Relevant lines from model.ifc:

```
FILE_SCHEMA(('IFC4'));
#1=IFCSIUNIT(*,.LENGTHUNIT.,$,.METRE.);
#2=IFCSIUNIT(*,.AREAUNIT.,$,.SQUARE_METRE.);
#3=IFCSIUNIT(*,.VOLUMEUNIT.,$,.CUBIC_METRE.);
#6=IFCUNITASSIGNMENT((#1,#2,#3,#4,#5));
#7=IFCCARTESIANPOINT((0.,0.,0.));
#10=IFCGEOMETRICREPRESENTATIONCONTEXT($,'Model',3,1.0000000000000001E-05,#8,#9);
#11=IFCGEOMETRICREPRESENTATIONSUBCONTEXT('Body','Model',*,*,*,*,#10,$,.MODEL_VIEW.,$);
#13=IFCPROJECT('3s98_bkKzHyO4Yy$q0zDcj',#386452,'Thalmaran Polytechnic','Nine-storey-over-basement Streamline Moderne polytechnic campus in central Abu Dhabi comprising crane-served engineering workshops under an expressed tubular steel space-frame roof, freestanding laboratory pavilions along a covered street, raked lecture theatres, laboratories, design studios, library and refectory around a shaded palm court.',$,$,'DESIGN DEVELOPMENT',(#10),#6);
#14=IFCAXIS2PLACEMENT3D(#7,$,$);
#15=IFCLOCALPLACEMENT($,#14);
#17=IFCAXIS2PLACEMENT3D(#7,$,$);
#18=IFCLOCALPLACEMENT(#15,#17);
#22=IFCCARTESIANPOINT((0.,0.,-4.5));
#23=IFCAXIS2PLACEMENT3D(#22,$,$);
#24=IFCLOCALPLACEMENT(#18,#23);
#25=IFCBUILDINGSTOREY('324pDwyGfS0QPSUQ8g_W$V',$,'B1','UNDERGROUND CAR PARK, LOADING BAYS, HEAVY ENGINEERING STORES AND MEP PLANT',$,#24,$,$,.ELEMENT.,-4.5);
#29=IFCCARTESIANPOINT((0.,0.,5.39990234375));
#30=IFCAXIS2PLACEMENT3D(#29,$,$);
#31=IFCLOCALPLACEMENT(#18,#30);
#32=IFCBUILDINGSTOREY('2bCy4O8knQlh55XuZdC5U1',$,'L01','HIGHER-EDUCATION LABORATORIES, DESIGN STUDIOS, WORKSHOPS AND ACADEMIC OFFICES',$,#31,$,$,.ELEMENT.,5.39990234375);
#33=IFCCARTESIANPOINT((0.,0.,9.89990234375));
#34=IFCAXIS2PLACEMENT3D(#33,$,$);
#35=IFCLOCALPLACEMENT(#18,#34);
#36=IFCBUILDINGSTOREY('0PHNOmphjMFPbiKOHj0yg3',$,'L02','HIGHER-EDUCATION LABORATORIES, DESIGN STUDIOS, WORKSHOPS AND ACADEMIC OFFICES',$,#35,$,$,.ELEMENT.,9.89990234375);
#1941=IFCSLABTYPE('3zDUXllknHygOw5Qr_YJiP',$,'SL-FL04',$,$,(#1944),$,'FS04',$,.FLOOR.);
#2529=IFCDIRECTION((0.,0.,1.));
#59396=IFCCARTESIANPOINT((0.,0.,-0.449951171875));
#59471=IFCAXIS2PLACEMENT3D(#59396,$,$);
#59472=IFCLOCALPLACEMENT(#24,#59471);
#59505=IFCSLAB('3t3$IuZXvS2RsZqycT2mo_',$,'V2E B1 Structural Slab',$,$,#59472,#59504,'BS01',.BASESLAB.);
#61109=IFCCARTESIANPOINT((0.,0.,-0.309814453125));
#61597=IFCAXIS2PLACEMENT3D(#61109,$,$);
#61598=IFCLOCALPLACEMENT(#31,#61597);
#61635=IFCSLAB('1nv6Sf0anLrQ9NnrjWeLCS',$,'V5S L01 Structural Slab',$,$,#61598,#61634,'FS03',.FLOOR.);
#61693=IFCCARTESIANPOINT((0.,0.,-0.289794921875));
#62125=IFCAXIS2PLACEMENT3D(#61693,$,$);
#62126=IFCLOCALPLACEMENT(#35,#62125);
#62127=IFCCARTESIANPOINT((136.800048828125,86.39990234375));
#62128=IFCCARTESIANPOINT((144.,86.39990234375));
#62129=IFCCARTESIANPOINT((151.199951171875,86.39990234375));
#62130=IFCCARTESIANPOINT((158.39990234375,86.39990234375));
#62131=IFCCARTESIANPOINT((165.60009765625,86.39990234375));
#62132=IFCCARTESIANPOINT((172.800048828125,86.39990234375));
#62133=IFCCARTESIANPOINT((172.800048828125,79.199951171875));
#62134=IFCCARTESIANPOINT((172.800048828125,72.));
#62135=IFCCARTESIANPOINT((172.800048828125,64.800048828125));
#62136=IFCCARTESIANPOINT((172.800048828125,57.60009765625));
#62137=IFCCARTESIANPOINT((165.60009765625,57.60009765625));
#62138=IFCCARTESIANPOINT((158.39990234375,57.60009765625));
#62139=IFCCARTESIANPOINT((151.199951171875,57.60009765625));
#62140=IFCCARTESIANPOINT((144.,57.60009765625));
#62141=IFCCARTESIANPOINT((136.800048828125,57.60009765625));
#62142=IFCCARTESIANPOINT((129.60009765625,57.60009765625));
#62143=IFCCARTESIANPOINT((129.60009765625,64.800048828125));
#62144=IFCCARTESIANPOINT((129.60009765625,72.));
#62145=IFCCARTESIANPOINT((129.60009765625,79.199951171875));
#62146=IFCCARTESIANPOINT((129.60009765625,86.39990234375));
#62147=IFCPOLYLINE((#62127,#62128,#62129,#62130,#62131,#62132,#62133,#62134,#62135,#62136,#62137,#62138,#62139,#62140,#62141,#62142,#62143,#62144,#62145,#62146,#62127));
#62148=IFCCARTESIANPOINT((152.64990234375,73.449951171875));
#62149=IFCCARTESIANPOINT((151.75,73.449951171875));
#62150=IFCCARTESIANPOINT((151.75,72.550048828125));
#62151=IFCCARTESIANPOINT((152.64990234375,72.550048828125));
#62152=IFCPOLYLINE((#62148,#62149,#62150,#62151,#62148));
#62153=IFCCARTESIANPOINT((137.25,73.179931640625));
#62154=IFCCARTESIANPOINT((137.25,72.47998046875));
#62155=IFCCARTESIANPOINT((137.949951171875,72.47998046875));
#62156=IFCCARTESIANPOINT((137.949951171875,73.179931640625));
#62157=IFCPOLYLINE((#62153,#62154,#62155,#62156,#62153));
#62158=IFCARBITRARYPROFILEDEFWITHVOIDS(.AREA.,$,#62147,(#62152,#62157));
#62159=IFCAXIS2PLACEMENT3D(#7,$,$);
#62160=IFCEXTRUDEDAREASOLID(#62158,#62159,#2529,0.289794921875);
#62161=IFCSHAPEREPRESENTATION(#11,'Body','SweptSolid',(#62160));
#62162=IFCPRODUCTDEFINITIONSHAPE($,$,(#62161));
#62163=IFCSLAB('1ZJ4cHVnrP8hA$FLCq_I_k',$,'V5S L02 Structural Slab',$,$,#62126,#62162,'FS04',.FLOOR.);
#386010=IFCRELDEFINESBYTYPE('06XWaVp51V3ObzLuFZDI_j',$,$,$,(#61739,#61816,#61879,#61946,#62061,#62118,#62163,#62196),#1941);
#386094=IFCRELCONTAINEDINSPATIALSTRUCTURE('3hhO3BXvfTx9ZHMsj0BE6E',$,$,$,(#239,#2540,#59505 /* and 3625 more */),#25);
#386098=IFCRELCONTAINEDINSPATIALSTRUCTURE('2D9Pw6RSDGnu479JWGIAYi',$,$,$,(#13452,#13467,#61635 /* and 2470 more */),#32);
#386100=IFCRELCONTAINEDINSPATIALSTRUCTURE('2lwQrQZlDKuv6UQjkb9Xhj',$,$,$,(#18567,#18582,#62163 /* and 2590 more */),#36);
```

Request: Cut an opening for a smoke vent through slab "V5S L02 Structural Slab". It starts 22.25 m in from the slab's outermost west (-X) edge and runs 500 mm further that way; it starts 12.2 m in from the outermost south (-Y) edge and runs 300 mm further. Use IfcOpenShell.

```python
import numpy as np
import ifcopenshell
import ifcopenshell.api.feature
import ifcopenshell.api.geometry
import ifcopenshell.api.root
import ifcopenshell.geom
import ifcopenshell.util.placement
import ifcopenshell.util.representation
import ifcopenshell.util.shape
import ifcopenshell.util.unit

model = ifcopenshell.open("model.ifc")
unit_scale = ifcopenshell.util.unit.calculate_unit_scale(model)
settings = ifcopenshell.geom.settings()


def volume(element):
    """Net volume in cubic metres, openings subtracted."""
    shape = ifcopenshell.geom.create_shape(settings, element)
    return ifcopenshell.util.shape.get_volume(shape.geometry)


slab = model.by_guid("1ZJ4cHVnrP8hA$FLCq_I_k")
before = volume(slab)

# Extent in the slab's own axes, in metres. The edges named are its -X and -Y sides.
slab_shape = ifcopenshell.geom.create_shape(settings, slab)
vertices = ifcopenshell.util.shape.get_vertices(slab_shape.geometry)
x_min, y_min, bottom = vertices.min(axis=0)
top = vertices[:, 2].max()

opening = ifcopenshell.api.root.create_entity(model, ifc_class="IfcOpeningElement", name="Smoke vent opening", predefined_type="OPENING")
context = ifcopenshell.util.representation.get_context(model, "Model", "Body", "MODEL_VIEW")
width, depth = 0.5, 0.3
outline = [(0.0, 0.0), (width, 0.0), (width, depth), (0.0, depth), (0.0, 0.0)]
# Overshoot both faces by 50 mm so the cut is clean.
shape = ifcopenshell.api.geometry.add_slab_representation(
    model, context=context, depth=top - bottom + 0.1, polyline=outline
)
ifcopenshell.api.geometry.assign_representation(model, product=opening, representation=shape)

matrix = ifcopenshell.util.placement.get_local_placement(slab.ObjectPlacement)
matrix[:, 3] = matrix @ np.append(np.array([x_min + 22.25, y_min + 12.2, bottom - 0.05]) / unit_scale, 1.0)
ifcopenshell.api.geometry.edit_object_placement(model, product=opening, matrix=matrix, is_si=False)
ifcopenshell.api.feature.add_feature(model, feature=opening, element=slab)

after = volume(slab)

print(f"slab volume {before:.3f} -> {after:.3f} m3")

model.write("model_v2.ifc")
```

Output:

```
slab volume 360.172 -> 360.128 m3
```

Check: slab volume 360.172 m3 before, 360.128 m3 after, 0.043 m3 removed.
